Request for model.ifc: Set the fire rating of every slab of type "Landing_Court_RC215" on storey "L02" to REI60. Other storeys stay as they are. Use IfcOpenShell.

First a look at what the model holds.

```python
import ifcopenshell
import ifcopenshell.util.element

model = ifcopenshell.open("model.ifc")
print(model.schema)
storey = next(s for s in model.by_type("IfcBuildingStorey") if s.Name == "L02")
slabs = [e for e in ifcopenshell.util.element.get_decomposition(storey) if e.is_a("IfcSlab")]
seen = {}
for e in slabs:
    element_type = ifcopenshell.util.element.get_type(e)
    key = (element_type.Name if element_type != e and element_type else None, ifcopenshell.util.element.get_pset(e, "Pset_SlabCommon", "FireRating"))
    seen[key] = seen.get(key, 0) + 1
for (name, value), count in sorted(seen.items(), key=str):
    print(count, "x", name, "|", value)
```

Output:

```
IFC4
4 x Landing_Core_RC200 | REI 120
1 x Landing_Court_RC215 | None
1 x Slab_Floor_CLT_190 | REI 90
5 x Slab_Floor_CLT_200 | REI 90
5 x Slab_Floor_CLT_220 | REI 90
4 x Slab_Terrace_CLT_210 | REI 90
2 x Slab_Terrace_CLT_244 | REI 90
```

```python
import ifcopenshell
import ifcopenshell.api.pset
import ifcopenshell.util.element

model = ifcopenshell.open("model.ifc")

storey = next(s for s in model.by_type("IfcBuildingStorey") if s.Name == "L02")
slabs = [e for e in ifcopenshell.util.element.get_decomposition(storey) if e.is_a("IfcSlab")]

count = 0
for e in slabs:
    element_type = ifcopenshell.util.element.get_type(e)
    if element_type in (None, e) or element_type.Name != "Landing_Court_RC215":
        continue
    # add_pset returns the element's existing set when there is one.
    pset = ifcopenshell.api.pset.add_pset(model, product=e, name="Pset_SlabCommon")
    ifcopenshell.api.pset.edit_pset(model, pset=pset, properties={"FireRating": "REI60"})
    count += 1

print(count, "slabs updated")

model.write("model_rev.ifc")
```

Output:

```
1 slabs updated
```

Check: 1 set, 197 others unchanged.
